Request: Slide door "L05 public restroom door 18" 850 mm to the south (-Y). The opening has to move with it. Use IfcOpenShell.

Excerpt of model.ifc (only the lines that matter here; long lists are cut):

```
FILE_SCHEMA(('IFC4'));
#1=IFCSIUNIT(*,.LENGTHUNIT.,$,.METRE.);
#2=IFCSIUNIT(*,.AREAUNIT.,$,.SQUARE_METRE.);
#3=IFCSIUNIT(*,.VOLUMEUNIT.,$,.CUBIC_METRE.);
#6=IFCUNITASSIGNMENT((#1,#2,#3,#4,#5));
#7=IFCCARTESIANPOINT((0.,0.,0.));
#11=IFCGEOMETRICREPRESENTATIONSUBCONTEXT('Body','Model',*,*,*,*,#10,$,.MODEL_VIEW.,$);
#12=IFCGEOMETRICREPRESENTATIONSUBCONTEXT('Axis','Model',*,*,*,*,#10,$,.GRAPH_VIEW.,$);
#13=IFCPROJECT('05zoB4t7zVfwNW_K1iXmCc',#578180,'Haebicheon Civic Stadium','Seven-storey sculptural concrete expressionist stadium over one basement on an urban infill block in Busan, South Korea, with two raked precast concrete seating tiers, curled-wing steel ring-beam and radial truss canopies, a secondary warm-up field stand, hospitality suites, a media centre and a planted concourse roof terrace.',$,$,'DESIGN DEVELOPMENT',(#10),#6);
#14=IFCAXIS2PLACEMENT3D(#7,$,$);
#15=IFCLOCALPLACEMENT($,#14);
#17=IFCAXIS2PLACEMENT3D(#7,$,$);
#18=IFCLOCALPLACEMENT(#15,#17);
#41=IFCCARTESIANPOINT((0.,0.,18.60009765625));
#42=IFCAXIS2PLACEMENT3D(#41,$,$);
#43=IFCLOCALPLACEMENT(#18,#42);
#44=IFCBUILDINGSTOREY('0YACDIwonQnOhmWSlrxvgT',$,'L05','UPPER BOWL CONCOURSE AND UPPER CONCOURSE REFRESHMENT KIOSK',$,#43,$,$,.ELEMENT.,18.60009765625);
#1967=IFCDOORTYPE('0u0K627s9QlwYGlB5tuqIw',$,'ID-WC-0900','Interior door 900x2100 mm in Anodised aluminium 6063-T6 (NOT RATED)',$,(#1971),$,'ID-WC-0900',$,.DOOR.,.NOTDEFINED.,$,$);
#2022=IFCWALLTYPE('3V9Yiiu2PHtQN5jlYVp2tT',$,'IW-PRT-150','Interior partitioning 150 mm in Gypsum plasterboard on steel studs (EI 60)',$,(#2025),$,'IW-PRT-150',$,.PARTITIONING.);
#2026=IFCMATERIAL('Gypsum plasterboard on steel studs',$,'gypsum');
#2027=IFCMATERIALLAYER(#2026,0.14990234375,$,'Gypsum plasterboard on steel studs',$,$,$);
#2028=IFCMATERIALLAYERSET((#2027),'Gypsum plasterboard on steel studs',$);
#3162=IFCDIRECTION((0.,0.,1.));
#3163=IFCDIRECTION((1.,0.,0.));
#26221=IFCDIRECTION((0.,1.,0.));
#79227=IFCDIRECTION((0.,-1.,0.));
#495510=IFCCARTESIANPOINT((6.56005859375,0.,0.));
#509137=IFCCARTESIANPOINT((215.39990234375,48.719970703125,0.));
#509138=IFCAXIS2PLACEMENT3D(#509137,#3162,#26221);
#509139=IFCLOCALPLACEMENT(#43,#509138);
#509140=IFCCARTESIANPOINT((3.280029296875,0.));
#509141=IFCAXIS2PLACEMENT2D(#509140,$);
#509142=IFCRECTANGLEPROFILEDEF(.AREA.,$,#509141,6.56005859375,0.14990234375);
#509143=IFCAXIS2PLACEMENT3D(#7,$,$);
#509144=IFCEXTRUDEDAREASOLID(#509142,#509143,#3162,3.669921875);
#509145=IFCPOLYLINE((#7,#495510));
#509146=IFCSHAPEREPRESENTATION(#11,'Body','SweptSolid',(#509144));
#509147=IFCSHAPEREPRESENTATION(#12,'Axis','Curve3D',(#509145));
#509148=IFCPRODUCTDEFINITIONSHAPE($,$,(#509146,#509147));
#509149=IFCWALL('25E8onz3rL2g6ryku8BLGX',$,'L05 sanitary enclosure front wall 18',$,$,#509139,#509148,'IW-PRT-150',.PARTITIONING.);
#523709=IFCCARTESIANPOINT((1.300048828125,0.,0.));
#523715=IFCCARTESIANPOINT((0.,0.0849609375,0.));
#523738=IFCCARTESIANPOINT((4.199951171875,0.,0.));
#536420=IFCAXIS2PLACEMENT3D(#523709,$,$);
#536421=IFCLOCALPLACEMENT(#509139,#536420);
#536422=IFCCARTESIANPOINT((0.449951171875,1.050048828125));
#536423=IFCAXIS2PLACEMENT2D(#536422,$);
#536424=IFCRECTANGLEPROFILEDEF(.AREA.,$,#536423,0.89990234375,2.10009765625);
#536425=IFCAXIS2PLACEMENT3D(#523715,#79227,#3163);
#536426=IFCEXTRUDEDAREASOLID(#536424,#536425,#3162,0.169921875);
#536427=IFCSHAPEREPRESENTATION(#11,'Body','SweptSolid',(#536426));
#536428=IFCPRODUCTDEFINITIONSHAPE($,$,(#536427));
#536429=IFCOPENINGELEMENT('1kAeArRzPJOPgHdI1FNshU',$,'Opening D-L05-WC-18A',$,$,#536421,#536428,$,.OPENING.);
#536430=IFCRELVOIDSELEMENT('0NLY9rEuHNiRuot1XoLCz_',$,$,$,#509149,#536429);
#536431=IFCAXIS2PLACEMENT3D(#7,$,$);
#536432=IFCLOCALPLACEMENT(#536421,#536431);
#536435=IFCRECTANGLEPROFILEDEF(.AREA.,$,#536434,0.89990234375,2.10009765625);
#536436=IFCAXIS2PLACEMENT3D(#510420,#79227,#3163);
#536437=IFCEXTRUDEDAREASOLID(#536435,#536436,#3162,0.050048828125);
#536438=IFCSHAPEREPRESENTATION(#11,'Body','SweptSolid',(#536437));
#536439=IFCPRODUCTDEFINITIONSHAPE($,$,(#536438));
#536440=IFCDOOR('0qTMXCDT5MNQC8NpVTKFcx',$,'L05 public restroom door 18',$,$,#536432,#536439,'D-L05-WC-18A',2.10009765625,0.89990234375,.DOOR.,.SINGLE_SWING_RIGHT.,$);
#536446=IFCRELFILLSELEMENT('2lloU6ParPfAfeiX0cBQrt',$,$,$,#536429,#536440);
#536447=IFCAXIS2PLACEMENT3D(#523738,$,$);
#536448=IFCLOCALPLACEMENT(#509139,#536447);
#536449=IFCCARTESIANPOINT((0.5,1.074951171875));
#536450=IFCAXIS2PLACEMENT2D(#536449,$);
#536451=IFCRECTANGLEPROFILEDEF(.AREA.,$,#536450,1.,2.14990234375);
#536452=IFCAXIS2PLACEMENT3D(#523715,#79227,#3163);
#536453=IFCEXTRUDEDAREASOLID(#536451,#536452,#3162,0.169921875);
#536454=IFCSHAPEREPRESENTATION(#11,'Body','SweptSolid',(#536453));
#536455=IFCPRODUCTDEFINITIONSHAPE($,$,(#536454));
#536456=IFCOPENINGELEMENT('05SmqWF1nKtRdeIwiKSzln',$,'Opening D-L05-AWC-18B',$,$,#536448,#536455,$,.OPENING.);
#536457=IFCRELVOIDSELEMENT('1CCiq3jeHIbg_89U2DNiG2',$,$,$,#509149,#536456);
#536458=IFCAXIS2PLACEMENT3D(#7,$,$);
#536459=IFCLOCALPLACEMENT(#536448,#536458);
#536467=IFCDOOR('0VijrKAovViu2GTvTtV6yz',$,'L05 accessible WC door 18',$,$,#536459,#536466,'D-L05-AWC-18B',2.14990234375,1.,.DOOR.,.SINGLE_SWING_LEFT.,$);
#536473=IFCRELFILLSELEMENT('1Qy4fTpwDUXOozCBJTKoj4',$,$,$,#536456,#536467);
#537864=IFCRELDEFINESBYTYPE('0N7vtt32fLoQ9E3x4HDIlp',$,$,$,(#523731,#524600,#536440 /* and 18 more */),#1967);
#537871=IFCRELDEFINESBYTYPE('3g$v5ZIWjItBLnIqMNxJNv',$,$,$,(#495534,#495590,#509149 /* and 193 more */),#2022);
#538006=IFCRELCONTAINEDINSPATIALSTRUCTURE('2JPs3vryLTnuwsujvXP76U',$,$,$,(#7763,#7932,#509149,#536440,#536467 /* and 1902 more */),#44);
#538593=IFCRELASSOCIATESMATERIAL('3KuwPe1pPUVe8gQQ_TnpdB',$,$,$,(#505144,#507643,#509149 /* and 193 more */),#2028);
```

```python
import ifcopenshell
import ifcopenshell.api.geometry
import ifcopenshell.util.placement
import ifcopenshell.util.unit

model = ifcopenshell.open("model.ifc")
unit_scale = ifcopenshell.util.unit.calculate_unit_scale(model)

door = model.by_id(536440)
opening = door.FillsVoids[0].RelatingOpeningElement
wall = opening.VoidsElements[0].RelatingBuildingElement

wall_matrix = ifcopenshell.util.placement.get_local_placement(wall.ObjectPlacement)
shift = wall_matrix[:3, 0] * -0.85 / unit_scale
before = ifcopenshell.util.placement.get_local_placement(door.ObjectPlacement)[:3, 3].copy()

# The door is placed relative to its opening, so it follows when the opening moves.
matrix = ifcopenshell.util.placement.get_local_placement(opening.ObjectPlacement)
matrix[:3, 3] += shift
ifcopenshell.api.geometry.edit_object_placement(
    model, product=opening, matrix=matrix, is_si=False, should_transform_children=True
)

after = ifcopenshell.util.placement.get_local_placement(door.ObjectPlacement)[:3, 3]
print("door moved by", (after - before).round(3) + 0.0)

model.write("model_rev.ifc")
```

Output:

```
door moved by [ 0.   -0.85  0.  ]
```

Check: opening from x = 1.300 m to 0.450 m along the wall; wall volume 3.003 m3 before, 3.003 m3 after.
